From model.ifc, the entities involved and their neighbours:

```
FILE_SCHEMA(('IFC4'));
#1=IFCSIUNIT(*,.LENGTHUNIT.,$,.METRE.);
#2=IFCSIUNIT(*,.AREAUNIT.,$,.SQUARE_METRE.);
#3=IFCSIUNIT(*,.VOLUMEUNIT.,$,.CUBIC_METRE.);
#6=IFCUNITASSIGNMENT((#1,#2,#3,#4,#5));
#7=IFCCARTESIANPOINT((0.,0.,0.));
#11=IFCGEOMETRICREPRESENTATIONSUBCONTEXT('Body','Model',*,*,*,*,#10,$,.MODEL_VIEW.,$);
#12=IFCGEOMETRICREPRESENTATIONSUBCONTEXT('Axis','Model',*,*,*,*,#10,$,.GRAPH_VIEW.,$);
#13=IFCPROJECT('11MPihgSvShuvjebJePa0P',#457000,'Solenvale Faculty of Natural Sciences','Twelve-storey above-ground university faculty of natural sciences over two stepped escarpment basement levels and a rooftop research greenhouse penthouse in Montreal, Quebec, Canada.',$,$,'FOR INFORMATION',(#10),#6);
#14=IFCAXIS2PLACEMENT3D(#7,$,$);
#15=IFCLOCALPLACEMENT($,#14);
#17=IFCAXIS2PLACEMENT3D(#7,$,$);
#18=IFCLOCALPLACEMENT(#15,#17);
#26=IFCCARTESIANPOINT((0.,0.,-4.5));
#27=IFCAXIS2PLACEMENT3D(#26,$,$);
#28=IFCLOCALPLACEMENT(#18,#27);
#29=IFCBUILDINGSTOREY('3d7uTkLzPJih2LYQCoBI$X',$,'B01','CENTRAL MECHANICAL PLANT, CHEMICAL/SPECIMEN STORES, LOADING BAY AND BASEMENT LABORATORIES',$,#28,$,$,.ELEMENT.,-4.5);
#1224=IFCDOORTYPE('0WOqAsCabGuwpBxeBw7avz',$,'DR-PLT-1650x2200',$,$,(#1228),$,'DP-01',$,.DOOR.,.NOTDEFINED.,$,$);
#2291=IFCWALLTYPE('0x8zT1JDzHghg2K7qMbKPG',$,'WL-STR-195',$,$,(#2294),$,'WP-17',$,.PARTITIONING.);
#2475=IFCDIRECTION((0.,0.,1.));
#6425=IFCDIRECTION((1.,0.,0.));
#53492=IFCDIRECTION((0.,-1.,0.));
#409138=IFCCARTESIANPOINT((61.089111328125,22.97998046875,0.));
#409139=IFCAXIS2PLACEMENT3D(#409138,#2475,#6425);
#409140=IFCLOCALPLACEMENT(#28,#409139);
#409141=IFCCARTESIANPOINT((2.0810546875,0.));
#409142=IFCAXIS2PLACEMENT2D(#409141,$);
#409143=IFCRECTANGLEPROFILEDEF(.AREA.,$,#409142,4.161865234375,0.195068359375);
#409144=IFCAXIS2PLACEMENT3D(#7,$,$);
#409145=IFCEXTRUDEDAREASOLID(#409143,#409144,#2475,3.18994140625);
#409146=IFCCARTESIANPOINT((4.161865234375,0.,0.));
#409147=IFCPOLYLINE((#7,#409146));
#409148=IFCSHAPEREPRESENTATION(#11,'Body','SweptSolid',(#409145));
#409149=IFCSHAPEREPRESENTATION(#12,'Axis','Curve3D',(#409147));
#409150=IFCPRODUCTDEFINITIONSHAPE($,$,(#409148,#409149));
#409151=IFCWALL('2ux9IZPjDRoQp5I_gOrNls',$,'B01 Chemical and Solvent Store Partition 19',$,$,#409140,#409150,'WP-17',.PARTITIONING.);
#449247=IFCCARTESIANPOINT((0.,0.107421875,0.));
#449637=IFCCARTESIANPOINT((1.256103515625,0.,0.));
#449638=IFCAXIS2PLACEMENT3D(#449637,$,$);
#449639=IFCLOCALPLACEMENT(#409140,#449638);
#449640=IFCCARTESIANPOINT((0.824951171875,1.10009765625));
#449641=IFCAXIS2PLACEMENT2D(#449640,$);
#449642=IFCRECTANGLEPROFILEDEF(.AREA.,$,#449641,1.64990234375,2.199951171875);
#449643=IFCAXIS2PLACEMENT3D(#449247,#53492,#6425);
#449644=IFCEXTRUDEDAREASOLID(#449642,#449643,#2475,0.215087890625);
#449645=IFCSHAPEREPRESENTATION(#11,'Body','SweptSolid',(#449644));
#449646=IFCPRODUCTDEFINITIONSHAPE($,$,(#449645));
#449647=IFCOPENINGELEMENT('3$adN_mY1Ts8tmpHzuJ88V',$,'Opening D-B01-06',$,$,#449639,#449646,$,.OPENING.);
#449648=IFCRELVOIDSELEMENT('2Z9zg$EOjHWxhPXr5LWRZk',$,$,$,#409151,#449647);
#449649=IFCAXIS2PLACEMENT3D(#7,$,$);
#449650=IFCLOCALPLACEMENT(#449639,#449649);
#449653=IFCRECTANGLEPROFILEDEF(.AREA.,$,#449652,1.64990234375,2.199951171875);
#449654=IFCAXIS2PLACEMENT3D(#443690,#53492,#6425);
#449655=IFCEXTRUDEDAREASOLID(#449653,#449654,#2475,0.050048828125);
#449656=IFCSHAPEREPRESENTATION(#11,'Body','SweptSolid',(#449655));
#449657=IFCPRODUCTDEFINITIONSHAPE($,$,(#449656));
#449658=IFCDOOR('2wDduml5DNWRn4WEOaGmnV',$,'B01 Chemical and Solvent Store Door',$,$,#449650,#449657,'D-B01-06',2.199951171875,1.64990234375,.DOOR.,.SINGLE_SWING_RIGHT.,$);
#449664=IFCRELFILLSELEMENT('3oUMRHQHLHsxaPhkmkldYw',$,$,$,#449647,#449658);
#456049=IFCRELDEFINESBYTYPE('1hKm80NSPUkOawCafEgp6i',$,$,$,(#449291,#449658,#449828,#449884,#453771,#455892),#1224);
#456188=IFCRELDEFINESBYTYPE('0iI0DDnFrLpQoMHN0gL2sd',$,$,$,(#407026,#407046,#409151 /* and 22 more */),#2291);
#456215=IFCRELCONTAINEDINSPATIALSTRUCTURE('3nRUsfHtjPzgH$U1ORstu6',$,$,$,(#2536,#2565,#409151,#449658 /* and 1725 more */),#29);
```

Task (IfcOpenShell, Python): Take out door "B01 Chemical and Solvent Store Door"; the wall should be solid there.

```python
import ifcopenshell
import ifcopenshell.api.feature
import ifcopenshell.api.root
import ifcopenshell.geom
import ifcopenshell.util.shape

model = ifcopenshell.open("model.ifc")
settings = ifcopenshell.geom.settings()


def volume(element):
    """Net volume in cubic metres, openings subtracted."""
    shape = ifcopenshell.geom.create_shape(settings, element)
    return ifcopenshell.util.shape.get_volume(shape.geometry)


door = model.by_guid("2wDduml5DNWRn4WEOaGmnV")
opening = door.FillsVoids[0].RelatingOpeningElement
wall = opening.VoidsElements[0].RelatingBuildingElement
before = volume(wall)

ifcopenshell.api.root.remove_product(model, product=door)
ifcopenshell.api.feature.remove_feature(model, feature=opening)

after = volume(wall)

print(f"wall volume {before:.3f} -> {after:.3f} m3")

model.write("model-out.ifc")
```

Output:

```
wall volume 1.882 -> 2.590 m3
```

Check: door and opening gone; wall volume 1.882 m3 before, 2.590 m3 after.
